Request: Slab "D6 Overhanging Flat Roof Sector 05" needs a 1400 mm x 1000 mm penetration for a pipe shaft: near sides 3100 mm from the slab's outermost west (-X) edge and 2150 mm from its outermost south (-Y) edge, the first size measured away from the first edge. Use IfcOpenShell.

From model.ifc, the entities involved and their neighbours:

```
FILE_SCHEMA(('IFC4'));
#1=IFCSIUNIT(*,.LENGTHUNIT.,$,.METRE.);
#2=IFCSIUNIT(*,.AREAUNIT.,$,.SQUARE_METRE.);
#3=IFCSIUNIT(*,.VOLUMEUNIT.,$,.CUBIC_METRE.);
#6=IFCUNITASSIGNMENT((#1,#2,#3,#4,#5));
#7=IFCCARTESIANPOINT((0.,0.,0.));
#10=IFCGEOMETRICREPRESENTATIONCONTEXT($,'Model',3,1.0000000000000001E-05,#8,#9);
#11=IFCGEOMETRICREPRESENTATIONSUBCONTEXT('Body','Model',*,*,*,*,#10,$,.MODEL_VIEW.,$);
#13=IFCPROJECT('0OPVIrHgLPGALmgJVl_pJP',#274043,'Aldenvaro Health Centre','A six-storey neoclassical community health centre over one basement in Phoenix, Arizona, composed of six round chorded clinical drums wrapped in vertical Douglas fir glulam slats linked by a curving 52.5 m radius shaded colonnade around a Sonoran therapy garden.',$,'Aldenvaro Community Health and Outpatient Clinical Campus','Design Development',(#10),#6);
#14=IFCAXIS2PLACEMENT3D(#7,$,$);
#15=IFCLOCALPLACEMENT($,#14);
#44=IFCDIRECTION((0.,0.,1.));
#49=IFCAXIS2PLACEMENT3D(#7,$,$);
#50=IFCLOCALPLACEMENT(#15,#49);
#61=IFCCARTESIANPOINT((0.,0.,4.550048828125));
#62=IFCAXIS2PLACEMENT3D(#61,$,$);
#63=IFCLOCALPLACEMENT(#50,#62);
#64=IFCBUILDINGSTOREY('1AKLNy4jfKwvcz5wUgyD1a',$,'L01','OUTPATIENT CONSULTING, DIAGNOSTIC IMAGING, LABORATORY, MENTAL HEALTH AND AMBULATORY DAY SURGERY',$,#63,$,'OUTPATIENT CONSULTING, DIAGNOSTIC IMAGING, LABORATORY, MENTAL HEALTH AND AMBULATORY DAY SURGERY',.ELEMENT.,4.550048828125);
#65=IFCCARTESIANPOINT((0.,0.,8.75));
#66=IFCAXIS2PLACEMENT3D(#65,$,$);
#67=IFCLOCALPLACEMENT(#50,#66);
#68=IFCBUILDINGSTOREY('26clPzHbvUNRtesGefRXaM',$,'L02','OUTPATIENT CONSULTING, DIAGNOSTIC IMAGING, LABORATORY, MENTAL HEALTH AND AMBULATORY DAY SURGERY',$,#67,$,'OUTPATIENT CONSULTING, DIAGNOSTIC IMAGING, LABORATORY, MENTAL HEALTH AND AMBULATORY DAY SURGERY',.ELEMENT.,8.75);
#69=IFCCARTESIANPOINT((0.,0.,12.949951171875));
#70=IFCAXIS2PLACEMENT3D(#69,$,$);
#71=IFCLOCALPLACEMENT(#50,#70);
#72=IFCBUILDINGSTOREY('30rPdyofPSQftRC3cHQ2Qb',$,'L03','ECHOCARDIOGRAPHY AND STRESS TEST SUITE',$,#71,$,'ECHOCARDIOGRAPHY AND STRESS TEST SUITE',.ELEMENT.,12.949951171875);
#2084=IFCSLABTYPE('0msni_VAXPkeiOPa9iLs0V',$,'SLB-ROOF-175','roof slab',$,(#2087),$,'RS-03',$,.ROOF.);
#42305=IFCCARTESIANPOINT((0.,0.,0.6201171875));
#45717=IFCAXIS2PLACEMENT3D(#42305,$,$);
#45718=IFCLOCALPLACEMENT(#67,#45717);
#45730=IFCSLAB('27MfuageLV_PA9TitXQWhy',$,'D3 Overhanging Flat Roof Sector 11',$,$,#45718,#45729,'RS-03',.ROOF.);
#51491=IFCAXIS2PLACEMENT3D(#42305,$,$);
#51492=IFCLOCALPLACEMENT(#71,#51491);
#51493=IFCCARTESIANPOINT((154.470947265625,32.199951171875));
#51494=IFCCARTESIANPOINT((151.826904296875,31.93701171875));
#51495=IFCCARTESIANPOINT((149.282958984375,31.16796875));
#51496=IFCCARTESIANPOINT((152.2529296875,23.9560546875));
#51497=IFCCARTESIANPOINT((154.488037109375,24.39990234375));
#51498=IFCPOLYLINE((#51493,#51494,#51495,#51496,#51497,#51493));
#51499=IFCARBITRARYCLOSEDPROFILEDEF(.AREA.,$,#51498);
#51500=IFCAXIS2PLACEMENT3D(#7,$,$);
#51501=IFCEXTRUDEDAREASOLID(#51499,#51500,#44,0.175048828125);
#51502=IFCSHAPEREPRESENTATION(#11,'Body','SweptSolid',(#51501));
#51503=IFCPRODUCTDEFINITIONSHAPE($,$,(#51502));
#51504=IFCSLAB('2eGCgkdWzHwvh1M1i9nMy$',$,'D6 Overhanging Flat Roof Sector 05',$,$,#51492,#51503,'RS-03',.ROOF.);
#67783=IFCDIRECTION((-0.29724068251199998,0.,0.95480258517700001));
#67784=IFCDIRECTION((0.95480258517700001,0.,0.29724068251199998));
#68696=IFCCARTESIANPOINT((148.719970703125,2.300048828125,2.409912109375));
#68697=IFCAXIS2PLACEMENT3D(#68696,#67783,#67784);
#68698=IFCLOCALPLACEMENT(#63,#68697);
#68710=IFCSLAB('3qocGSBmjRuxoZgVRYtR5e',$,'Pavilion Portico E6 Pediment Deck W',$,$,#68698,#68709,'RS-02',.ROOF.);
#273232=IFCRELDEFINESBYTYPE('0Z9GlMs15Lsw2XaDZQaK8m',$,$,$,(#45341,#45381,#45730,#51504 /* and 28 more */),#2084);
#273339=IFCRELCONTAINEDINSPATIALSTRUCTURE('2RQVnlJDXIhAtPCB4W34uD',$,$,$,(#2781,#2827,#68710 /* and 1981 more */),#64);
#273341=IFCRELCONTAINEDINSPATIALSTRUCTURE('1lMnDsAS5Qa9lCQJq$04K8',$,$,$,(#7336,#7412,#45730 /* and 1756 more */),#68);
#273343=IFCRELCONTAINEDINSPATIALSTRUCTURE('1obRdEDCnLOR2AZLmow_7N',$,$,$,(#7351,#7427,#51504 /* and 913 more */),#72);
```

```python
import numpy as np
import ifcopenshell
import ifcopenshell.api.feature
import ifcopenshell.api.geometry
import ifcopenshell.api.root
import ifcopenshell.geom
import ifcopenshell.util.placement
import ifcopenshell.util.representation
import ifcopenshell.util.shape
import ifcopenshell.util.unit

model = ifcopenshell.open("model.ifc")
unit_scale = ifcopenshell.util.unit.calculate_unit_scale(model)
settings = ifcopenshell.geom.settings()


def volume(element):
    """Net volume in cubic metres, openings subtracted."""
    shape = ifcopenshell.geom.create_shape(settings, element)
    return ifcopenshell.util.shape.get_volume(shape.geometry)


slab = model.by_guid("2eGCgkdWzHwvh1M1i9nMy$")
before = volume(slab)

# Extent in the slab's own axes, in metres. The edges named are its -X and -Y sides.
slab_shape = ifcopenshell.geom.create_shape(settings, slab)
vertices = ifcopenshell.util.shape.get_vertices(slab_shape.geometry)
x_min, y_min, bottom = vertices.min(axis=0)
top = vertices[:, 2].max()

opening = ifcopenshell.api.root.create_entity(model, ifc_class="IfcOpeningElement", name="Pipe shaft opening", predefined_type="OPENING")
context = ifcopenshell.util.representation.get_context(model, "Model", "Body", "MODEL_VIEW")
width, depth = 1.4, 1
outline = [(0.0, 0.0), (width, 0.0), (width, depth), (0.0, depth), (0.0, 0.0)]
# Overshoot both faces by 50 mm so the cut is clean.
shape = ifcopenshell.api.geometry.add_slab_representation(
    model, context=context, depth=top - bottom + 0.1, polyline=outline
)
ifcopenshell.api.geometry.assign_representation(model, product=opening, representation=shape)

matrix = ifcopenshell.util.placement.get_local_placement(slab.ObjectPlacement)
matrix[:, 3] = matrix @ np.append(np.array([x_min + 3.1, y_min + 2.15, bottom - 0.05]) / unit_scale, 1.0)
ifcopenshell.api.geometry.edit_object_placement(model, product=opening, matrix=matrix, is_si=False)
ifcopenshell.api.feature.add_feature(model, feature=opening, element=slab)

after = volume(slab)

print(f"slab volume {before:.3f} -> {after:.3f} m3")

model.write("model_updated.ifc")
```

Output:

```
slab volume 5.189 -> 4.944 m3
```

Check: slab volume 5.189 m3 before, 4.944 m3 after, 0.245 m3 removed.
